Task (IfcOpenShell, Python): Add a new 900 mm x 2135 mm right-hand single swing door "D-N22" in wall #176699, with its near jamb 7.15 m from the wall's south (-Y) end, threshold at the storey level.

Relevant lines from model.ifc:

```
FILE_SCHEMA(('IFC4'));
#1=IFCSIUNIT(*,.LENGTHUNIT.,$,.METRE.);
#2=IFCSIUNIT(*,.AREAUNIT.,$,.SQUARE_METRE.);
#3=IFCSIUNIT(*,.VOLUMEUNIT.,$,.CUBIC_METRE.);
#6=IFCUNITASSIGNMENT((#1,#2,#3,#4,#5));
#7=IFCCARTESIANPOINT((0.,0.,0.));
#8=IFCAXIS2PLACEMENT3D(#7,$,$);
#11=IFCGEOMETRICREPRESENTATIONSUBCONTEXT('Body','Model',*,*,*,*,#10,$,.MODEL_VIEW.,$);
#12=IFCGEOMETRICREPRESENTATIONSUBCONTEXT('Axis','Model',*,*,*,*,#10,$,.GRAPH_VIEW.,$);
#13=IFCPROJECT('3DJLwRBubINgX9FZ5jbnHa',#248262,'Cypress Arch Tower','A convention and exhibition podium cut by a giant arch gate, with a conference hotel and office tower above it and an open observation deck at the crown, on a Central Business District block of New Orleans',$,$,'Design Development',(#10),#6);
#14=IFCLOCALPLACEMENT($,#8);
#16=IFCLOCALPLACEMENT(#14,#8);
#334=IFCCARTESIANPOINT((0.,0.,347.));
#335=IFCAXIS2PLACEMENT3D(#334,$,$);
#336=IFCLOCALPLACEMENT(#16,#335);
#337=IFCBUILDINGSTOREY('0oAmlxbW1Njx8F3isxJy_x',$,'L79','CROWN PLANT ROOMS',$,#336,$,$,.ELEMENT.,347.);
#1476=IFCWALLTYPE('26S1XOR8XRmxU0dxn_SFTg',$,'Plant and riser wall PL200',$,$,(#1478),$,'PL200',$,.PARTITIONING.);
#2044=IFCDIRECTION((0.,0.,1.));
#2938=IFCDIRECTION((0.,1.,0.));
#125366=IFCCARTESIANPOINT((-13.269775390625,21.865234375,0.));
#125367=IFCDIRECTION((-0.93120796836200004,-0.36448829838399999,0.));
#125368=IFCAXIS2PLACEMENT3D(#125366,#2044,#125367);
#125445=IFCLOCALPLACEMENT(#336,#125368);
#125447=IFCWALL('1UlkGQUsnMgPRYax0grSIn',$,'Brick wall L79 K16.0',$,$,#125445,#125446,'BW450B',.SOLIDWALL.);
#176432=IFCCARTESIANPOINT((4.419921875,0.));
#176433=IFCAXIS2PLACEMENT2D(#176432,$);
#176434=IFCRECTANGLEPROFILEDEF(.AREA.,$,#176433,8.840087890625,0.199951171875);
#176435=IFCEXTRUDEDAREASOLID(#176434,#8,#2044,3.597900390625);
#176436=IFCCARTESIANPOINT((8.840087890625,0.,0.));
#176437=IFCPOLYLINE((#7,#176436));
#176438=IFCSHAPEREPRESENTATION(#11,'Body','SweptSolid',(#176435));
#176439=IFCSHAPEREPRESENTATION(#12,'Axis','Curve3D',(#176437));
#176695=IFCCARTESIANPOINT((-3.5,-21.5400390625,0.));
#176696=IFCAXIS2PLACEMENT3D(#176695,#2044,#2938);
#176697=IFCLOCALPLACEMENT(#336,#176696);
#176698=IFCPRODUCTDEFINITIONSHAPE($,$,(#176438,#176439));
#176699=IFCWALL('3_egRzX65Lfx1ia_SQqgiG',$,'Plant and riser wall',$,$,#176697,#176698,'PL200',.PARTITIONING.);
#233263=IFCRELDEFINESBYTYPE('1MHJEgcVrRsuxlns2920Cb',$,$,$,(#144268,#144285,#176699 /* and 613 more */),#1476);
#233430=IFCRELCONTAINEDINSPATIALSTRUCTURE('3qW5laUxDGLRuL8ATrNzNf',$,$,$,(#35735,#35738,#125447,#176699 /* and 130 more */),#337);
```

```python
import numpy as np
import ifcopenshell
import ifcopenshell.api.feature
import ifcopenshell.api.geometry
import ifcopenshell.api.root
import ifcopenshell.api.spatial
import ifcopenshell.geom
import ifcopenshell.util.element
import ifcopenshell.util.placement
import ifcopenshell.util.representation
import ifcopenshell.util.shape
import ifcopenshell.util.unit

model = ifcopenshell.open("model.ifc")
unit_scale = ifcopenshell.util.unit.calculate_unit_scale(model)
settings = ifcopenshell.geom.settings()


def volume(element):
    """Net volume in cubic metres, openings subtracted."""
    shape = ifcopenshell.geom.create_shape(settings, element)
    return ifcopenshell.util.shape.get_volume(shape.geometry)


wall = model.by_guid("3_egRzX65Lfx1ia_SQqgiG")
storey = ifcopenshell.util.element.get_container(wall, ifc_class="IfcBuildingStorey")
context = ifcopenshell.util.representation.get_context(model, "Model", "Body", "MODEL_VIEW")
before = volume(wall)

width, height, from_end, sill = 0.9, 2.135, 7.15, 0.0  # metres

# The wall runs along its own X axis, and the end named is its -X end.
wall_shape = ifcopenshell.geom.create_shape(settings, wall)
x, y, z = ifcopenshell.util.shape.get_vertices(wall_shape.geometry).T
start = x.min() + from_end
face, thickness = float(y.min()), float(y.max() - y.min())
wall_matrix = ifcopenshell.util.placement.get_local_placement(wall.ObjectPlacement)
level = ifcopenshell.util.placement.get_local_placement(storey.ObjectPlacement)[2, 3]


def in_wall(x, y):
    """Placement at x, y metres in the wall's axes, at sill height."""
    matrix = wall_matrix.copy()
    matrix[:, 3] = wall_matrix @ np.array([x / unit_scale, y / unit_scale, 0.0, 1.0])
    matrix[2, 3] = level + sill / unit_scale
    return matrix


# Opening: a box that overshoots both wall faces by 50 mm.
opening = ifcopenshell.api.root.create_entity(model, ifc_class="IfcOpeningElement", predefined_type="OPENING")
box = ifcopenshell.api.geometry.add_wall_representation(
    model, context=context, length=width, height=height, thickness=thickness + 0.1
)
ifcopenshell.api.geometry.assign_representation(model, product=opening, representation=box)
ifcopenshell.api.geometry.edit_object_placement(model, product=opening, matrix=in_wall(start, face - 0.05), is_si=False)
ifcopenshell.api.feature.add_feature(model, feature=opening, element=wall)

door = ifcopenshell.api.root.create_entity(model, ifc_class="IfcDoor", name="D-N22", predefined_type="DOOR")
door.OverallWidth, door.OverallHeight = width / unit_scale, height / unit_scale
door.OperationType = "SINGLE_SWING_RIGHT"
body = ifcopenshell.api.geometry.add_door_representation(
    model,
    context=context,
    overall_width=door.OverallWidth,
    overall_height=door.OverallHeight,
    operation_type="SINGLE_SWING_RIGHT",
    lining_properties={"LiningDepth": thickness / unit_scale, "ThresholdDepth": thickness / unit_scale},
)
ifcopenshell.api.geometry.assign_representation(model, product=door, representation=body)
ifcopenshell.api.spatial.assign_container(model, products=[door], relating_structure=storey)
ifcopenshell.api.feature.add_filling(model, opening=opening, element=door)

# The lining spans the wall, so the door starts at the wall face.
ifcopenshell.api.geometry.edit_object_placement(model, product=door, matrix=in_wall(start, face), is_si=False)

after = volume(wall)

print(f"wall volume {before:.3f} -> {after:.3f} m3")

model.write("model_v2.ifc")
```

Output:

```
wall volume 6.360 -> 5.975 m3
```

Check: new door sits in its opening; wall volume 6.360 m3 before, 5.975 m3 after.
